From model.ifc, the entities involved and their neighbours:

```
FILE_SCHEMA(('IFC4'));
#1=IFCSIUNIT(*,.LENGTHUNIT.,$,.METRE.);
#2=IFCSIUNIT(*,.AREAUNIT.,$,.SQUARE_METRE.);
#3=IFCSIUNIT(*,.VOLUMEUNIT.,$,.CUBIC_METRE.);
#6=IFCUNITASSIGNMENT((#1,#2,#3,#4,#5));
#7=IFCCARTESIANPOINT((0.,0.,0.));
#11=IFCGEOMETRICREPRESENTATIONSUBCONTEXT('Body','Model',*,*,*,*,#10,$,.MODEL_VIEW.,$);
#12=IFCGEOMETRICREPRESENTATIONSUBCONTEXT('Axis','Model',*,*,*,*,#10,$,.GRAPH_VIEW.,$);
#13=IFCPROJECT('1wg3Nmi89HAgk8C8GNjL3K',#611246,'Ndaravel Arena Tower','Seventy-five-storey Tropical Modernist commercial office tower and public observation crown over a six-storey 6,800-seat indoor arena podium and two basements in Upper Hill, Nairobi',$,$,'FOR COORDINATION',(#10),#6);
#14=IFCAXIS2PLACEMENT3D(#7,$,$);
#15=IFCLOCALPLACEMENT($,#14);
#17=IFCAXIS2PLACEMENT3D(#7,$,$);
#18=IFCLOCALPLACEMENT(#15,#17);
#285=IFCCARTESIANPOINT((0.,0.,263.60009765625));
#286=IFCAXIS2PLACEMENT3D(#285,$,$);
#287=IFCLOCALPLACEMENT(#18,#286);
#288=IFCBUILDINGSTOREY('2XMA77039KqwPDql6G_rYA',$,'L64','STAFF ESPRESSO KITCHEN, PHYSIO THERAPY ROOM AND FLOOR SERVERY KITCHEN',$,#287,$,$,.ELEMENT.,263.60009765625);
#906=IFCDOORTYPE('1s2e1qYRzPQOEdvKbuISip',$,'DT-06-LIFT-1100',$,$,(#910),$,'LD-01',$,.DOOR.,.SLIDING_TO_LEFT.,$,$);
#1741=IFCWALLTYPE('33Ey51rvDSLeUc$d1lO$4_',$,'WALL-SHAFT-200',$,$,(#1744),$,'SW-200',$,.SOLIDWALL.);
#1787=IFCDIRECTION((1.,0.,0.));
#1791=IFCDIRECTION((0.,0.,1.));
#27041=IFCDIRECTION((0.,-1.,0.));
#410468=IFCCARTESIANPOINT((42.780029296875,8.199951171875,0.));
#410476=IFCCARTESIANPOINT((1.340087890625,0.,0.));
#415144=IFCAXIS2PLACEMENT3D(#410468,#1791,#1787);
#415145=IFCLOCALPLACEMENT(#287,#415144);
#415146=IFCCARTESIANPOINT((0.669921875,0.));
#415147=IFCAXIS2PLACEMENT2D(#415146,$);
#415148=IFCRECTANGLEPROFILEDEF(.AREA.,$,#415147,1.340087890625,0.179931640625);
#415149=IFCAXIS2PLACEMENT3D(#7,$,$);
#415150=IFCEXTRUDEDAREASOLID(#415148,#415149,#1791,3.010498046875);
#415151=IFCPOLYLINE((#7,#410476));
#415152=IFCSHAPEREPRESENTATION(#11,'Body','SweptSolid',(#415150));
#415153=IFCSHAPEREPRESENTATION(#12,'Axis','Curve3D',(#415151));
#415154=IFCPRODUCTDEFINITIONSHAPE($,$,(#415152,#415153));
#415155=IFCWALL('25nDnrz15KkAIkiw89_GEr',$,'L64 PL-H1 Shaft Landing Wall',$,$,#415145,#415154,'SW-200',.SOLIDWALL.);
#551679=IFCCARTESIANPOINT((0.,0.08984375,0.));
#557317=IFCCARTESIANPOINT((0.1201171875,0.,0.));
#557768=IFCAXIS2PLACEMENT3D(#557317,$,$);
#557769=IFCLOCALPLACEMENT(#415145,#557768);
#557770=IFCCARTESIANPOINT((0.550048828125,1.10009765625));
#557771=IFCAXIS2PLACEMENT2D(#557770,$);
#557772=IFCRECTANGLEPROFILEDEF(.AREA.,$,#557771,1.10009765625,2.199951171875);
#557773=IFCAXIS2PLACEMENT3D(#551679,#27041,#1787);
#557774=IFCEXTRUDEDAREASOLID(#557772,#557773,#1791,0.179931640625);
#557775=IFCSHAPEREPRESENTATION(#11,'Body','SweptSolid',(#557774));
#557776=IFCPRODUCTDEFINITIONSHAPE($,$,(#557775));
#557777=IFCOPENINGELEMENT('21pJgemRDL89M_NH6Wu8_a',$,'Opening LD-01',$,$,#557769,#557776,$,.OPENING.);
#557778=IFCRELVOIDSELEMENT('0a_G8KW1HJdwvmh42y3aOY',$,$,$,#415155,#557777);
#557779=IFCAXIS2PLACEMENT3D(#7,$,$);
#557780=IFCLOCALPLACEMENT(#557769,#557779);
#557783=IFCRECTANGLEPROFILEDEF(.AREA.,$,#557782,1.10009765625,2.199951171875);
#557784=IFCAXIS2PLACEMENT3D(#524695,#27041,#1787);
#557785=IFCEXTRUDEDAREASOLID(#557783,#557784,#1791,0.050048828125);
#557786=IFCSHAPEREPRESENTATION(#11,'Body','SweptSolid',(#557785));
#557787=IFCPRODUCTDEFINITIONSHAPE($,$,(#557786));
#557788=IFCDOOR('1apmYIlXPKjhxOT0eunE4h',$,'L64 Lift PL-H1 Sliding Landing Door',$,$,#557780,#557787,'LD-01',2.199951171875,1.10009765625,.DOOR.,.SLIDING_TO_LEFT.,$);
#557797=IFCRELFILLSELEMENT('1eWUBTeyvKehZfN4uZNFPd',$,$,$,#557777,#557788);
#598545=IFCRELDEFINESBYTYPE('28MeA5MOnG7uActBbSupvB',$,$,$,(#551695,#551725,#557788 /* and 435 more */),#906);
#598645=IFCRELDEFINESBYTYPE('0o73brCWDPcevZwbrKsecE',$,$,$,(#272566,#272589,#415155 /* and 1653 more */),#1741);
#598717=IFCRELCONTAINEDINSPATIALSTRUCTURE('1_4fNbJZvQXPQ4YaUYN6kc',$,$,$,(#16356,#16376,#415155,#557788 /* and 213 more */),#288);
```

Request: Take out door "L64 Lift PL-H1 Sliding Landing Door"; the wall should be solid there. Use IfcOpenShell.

```python
import ifcopenshell
import ifcopenshell.api.feature
import ifcopenshell.api.root
import ifcopenshell.geom
import ifcopenshell.util.shape

model = ifcopenshell.open("model.ifc")
settings = ifcopenshell.geom.settings()


def volume(element):
    """Net volume in cubic metres, openings subtracted."""
    shape = ifcopenshell.geom.create_shape(settings, element)
    return ifcopenshell.util.shape.get_volume(shape.geometry)


door = model.by_id(557788)
opening = door.FillsVoids[0].RelatingOpeningElement
wall = opening.VoidsElements[0].RelatingBuildingElement
before = volume(wall)

ifcopenshell.api.root.remove_product(model, product=door)
ifcopenshell.api.feature.remove_feature(model, feature=opening)

after = volume(wall)

print(f"wall volume {before:.3f} -> {after:.3f} m3")

model.write("model-out.ifc")
```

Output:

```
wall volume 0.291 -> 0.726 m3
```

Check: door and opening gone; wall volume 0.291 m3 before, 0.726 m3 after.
